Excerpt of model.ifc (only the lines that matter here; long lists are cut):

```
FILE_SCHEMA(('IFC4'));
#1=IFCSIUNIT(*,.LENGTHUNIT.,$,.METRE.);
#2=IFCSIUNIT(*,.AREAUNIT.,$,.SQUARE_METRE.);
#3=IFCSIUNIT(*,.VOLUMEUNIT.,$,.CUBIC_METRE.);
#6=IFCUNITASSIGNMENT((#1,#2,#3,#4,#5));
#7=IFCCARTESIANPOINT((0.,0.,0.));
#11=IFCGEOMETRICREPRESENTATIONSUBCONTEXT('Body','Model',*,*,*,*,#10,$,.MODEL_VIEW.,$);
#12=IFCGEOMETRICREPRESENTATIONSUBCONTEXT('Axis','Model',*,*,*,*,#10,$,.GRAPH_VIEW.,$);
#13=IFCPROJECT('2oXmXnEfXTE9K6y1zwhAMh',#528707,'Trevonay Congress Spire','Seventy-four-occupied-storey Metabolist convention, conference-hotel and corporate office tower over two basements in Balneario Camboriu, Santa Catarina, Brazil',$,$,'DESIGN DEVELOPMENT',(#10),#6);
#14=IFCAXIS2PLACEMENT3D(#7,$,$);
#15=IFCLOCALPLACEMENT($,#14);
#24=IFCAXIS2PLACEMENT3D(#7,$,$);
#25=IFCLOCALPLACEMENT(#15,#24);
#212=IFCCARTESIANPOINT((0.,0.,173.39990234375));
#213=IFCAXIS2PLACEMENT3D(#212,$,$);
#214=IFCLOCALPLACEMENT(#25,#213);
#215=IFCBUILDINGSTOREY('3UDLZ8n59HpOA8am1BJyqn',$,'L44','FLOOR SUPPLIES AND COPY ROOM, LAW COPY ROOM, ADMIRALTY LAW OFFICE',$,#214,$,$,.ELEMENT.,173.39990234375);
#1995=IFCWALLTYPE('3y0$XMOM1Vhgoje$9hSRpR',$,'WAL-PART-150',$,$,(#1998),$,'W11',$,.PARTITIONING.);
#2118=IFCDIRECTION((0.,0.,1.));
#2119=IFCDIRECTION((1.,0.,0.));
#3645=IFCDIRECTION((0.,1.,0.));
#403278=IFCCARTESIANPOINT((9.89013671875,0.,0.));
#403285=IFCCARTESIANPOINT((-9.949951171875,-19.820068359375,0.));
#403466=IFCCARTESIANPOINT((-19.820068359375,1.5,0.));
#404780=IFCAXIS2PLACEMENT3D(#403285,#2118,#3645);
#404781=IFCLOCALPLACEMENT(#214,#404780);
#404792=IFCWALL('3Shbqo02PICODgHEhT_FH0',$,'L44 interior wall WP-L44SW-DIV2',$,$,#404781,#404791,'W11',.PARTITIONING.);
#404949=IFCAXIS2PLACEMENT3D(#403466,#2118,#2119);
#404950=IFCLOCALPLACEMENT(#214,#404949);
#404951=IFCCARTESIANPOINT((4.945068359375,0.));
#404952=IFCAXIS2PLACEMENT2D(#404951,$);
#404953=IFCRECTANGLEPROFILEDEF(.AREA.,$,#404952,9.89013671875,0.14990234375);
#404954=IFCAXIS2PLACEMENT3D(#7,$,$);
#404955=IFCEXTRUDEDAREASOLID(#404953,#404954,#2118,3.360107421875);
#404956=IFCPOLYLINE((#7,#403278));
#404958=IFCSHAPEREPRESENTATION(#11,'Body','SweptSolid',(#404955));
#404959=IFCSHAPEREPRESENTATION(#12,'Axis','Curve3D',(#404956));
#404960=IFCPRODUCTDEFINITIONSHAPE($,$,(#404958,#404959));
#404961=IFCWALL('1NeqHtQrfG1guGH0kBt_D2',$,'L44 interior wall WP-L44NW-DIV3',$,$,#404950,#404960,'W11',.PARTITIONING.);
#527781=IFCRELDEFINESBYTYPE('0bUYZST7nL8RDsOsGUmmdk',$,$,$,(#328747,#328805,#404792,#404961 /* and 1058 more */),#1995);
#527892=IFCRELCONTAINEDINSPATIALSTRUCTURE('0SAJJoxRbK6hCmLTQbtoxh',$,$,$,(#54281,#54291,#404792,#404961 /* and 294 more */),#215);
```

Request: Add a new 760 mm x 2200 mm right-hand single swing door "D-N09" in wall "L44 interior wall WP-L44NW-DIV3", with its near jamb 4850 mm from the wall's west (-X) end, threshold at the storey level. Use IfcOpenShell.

```python
import numpy as np
import ifcopenshell
import ifcopenshell.api.feature
import ifcopenshell.api.geometry
import ifcopenshell.api.root
import ifcopenshell.api.spatial
import ifcopenshell.geom
import ifcopenshell.util.element
import ifcopenshell.util.placement
import ifcopenshell.util.representation
import ifcopenshell.util.shape
import ifcopenshell.util.unit

model = ifcopenshell.open("model.ifc")
unit_scale = ifcopenshell.util.unit.calculate_unit_scale(model)
settings = ifcopenshell.geom.settings()


def volume(element):
    """Net volume in cubic metres, openings subtracted."""
    shape = ifcopenshell.geom.create_shape(settings, element)
    return ifcopenshell.util.shape.get_volume(shape.geometry)


wall = model.by_guid("1NeqHtQrfG1guGH0kBt_D2")
storey = ifcopenshell.util.element.get_container(wall, ifc_class="IfcBuildingStorey")
context = ifcopenshell.util.representation.get_context(model, "Model", "Body", "MODEL_VIEW")
before = volume(wall)

width, height, from_end, sill = 0.76, 2.2, 4.85, 0.0  # metres

# The wall runs along its own X axis, and the end named is its -X end.
wall_shape = ifcopenshell.geom.create_shape(settings, wall)
x, y, z = ifcopenshell.util.shape.get_vertices(wall_shape.geometry).T
start = x.min() + from_end
face, thickness = float(y.min()), float(y.max() - y.min())
wall_matrix = ifcopenshell.util.placement.get_local_placement(wall.ObjectPlacement)
level = ifcopenshell.util.placement.get_local_placement(storey.ObjectPlacement)[2, 3]


def in_wall(x, y):
    """Placement at x, y metres in the wall's axes, at sill height."""
    matrix = wall_matrix.copy()
    matrix[:, 3] = wall_matrix @ np.array([x / unit_scale, y / unit_scale, 0.0, 1.0])
    matrix[2, 3] = level + sill / unit_scale
    return matrix


# Opening: a box that overshoots both wall faces by 50 mm.
opening = ifcopenshell.api.root.create_entity(model, ifc_class="IfcOpeningElement", predefined_type="OPENING")
box = ifcopenshell.api.geometry.add_wall_representation(
    model, context=context, length=width, height=height, thickness=thickness + 0.1
)
ifcopenshell.api.geometry.assign_representation(model, product=opening, representation=box)
ifcopenshell.api.geometry.edit_object_placement(model, product=opening, matrix=in_wall(start, face - 0.05), is_si=False)
ifcopenshell.api.feature.add_feature(model, feature=opening, element=wall)

door = ifcopenshell.api.root.create_entity(model, ifc_class="IfcDoor", name="D-N09", predefined_type="DOOR")
door.OverallWidth, door.OverallHeight = width / unit_scale, height / unit_scale
door.OperationType = "SINGLE_SWING_RIGHT"
body = ifcopenshell.api.geometry.add_door_representation(
    model,
    context=context,
    overall_width=door.OverallWidth,
    overall_height=door.OverallHeight,
    operation_type="SINGLE_SWING_RIGHT",
    lining_properties={"LiningDepth": thickness / unit_scale, "ThresholdDepth": thickness / unit_scale},
)
ifcopenshell.api.geometry.assign_representation(model, product=door, representation=body)
ifcopenshell.api.spatial.assign_container(model, products=[door], relating_structure=storey)
ifcopenshell.api.feature.add_filling(model, opening=opening, element=door)

# The lining spans the wall, so the door starts at the wall face.
ifcopenshell.api.geometry.edit_object_placement(model, product=door, matrix=in_wall(start, face), is_si=False)

after = volume(wall)

print(f"wall volume {before:.3f} -> {after:.3f} m3")

model.write("model_rev.ifc")
```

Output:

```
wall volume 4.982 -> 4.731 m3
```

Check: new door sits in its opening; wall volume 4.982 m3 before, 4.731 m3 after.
